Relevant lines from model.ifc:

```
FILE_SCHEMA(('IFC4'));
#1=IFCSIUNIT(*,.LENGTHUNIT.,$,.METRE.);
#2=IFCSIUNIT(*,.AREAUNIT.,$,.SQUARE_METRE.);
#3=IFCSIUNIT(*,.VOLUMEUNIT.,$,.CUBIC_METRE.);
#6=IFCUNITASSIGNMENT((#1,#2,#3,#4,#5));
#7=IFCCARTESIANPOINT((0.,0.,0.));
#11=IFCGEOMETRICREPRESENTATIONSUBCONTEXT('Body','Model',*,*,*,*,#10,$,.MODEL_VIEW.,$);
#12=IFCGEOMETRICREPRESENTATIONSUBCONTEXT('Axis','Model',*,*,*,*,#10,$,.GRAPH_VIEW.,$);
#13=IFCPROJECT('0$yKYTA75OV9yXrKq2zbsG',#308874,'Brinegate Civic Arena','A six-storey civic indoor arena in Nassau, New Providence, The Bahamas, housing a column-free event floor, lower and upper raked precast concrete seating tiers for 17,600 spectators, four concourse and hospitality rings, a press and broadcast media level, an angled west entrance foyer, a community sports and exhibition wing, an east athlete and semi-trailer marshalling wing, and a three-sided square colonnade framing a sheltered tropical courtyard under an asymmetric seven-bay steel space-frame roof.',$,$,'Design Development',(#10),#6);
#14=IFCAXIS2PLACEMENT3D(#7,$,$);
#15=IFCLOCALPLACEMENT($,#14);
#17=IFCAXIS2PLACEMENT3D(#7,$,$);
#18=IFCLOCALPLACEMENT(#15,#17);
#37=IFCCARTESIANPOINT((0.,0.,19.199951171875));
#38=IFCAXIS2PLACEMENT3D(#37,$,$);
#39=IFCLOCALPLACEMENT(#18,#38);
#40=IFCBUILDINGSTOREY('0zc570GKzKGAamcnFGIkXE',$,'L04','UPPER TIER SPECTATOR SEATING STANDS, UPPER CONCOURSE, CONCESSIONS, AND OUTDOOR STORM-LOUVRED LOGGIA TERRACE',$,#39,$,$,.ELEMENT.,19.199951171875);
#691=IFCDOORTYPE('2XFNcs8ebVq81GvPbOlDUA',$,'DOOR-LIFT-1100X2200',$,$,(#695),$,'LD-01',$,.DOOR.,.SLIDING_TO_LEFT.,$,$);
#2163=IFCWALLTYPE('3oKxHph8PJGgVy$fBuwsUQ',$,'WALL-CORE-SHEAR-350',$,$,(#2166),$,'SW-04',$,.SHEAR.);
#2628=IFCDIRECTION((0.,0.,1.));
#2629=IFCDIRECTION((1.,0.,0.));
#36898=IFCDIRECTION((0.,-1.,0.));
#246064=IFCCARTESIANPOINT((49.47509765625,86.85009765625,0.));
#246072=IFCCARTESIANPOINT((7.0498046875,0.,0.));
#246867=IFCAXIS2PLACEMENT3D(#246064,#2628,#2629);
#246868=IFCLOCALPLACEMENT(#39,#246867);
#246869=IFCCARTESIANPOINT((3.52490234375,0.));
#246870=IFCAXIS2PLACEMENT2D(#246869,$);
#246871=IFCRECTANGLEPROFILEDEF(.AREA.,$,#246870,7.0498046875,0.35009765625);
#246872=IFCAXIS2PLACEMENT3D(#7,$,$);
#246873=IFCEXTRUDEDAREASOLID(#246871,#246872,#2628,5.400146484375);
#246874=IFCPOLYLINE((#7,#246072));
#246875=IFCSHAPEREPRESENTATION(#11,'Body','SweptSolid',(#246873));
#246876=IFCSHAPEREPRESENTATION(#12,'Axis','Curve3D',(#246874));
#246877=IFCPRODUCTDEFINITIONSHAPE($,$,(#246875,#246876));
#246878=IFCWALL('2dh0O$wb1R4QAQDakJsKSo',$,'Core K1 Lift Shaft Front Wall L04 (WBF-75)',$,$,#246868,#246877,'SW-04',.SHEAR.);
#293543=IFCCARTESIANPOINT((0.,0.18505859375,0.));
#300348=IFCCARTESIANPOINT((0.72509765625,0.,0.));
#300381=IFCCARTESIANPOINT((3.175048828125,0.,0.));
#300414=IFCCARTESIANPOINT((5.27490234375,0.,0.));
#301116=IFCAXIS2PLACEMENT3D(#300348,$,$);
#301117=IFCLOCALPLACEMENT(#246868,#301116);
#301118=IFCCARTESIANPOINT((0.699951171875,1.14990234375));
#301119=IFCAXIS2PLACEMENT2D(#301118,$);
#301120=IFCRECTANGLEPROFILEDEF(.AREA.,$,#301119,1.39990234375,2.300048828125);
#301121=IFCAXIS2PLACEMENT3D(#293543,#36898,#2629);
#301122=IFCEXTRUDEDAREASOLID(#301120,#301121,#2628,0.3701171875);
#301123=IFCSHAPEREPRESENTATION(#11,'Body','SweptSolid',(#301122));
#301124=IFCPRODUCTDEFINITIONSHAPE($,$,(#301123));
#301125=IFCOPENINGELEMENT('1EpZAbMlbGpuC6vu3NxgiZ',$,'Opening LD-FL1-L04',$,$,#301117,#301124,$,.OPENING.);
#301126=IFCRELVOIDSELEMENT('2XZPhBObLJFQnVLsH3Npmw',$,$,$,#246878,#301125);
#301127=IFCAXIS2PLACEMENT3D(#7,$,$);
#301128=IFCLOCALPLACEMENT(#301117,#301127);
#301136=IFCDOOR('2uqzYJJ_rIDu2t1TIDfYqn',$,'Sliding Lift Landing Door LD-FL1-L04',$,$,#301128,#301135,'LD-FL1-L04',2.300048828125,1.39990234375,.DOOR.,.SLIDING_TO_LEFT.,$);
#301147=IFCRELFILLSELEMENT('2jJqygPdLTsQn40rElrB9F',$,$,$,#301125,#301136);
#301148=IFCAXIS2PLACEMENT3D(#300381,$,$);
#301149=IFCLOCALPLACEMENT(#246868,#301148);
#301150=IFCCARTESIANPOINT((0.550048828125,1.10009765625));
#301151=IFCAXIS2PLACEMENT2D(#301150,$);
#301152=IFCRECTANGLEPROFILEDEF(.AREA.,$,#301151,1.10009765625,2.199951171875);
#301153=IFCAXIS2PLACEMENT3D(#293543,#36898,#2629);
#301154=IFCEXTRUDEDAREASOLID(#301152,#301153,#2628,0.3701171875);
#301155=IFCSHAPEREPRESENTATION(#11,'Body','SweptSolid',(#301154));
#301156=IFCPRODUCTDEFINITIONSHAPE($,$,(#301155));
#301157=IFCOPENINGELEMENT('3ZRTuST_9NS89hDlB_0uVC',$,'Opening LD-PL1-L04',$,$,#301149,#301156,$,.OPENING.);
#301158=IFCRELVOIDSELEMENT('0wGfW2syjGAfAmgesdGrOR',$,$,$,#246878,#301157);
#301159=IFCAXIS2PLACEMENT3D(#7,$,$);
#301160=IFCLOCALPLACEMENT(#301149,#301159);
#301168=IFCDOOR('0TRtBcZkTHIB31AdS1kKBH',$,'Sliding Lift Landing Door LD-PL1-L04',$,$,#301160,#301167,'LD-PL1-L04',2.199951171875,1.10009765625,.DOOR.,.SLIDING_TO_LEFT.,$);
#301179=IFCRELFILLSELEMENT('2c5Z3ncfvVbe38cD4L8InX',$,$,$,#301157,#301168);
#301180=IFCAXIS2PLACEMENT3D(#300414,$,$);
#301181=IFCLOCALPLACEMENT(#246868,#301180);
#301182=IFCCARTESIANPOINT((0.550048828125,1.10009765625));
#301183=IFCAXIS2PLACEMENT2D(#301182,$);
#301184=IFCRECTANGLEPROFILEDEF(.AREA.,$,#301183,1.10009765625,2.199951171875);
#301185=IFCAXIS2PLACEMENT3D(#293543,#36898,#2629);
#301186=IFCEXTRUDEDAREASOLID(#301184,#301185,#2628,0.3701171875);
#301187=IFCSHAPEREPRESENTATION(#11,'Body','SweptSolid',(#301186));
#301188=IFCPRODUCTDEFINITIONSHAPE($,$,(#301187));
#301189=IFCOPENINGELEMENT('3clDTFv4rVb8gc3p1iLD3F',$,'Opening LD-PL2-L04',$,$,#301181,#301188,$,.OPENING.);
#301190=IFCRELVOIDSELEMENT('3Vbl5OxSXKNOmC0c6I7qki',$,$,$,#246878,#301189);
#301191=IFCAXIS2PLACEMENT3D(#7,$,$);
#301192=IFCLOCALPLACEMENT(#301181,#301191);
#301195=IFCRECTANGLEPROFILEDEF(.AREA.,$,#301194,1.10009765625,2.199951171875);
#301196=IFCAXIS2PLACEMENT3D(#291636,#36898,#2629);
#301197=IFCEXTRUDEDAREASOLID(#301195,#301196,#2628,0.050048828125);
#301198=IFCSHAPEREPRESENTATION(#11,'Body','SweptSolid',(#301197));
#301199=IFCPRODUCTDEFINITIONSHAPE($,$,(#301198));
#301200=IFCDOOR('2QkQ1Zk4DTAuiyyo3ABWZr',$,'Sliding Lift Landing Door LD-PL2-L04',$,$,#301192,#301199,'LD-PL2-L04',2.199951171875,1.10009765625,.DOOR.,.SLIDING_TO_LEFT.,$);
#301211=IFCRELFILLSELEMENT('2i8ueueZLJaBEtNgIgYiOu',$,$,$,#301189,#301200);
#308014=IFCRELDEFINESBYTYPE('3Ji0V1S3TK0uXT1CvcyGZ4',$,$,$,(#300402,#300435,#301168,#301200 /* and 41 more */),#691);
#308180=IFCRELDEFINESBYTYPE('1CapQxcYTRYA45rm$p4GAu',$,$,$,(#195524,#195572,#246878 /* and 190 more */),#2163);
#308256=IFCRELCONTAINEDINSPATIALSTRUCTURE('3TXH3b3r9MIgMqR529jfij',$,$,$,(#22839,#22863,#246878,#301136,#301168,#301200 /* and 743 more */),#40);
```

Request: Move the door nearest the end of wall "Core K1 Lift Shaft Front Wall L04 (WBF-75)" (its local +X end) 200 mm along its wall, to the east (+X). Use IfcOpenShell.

```python
import ifcopenshell
import ifcopenshell.api.geometry
import ifcopenshell.util.placement

model = ifcopenshell.open("model.ifc")

door = model.by_guid("2QkQ1Zk4DTAuiyyo3ABWZr")
opening = door.FillsVoids[0].RelatingOpeningElement
wall = opening.VoidsElements[0].RelatingBuildingElement

wall_matrix = ifcopenshell.util.placement.get_local_placement(wall.ObjectPlacement)
shift = wall_matrix[:3, 0] * 0.2
before = ifcopenshell.util.placement.get_local_placement(door.ObjectPlacement)[:3, 3].copy()

# The door is placed relative to its opening, so it follows when the opening moves.
matrix = ifcopenshell.util.placement.get_local_placement(opening.ObjectPlacement)
matrix[:3, 3] += shift
ifcopenshell.api.geometry.edit_object_placement(
    model, product=opening, matrix=matrix, is_si=False, should_transform_children=True
)

after = ifcopenshell.util.placement.get_local_placement(door.ObjectPlacement)[:3, 3]
print("door moved by", (after - before).round(3) + 0.0)

model.write("model_updated.ifc")
```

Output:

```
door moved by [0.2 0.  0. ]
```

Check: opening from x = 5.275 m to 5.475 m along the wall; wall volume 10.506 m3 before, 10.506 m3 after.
